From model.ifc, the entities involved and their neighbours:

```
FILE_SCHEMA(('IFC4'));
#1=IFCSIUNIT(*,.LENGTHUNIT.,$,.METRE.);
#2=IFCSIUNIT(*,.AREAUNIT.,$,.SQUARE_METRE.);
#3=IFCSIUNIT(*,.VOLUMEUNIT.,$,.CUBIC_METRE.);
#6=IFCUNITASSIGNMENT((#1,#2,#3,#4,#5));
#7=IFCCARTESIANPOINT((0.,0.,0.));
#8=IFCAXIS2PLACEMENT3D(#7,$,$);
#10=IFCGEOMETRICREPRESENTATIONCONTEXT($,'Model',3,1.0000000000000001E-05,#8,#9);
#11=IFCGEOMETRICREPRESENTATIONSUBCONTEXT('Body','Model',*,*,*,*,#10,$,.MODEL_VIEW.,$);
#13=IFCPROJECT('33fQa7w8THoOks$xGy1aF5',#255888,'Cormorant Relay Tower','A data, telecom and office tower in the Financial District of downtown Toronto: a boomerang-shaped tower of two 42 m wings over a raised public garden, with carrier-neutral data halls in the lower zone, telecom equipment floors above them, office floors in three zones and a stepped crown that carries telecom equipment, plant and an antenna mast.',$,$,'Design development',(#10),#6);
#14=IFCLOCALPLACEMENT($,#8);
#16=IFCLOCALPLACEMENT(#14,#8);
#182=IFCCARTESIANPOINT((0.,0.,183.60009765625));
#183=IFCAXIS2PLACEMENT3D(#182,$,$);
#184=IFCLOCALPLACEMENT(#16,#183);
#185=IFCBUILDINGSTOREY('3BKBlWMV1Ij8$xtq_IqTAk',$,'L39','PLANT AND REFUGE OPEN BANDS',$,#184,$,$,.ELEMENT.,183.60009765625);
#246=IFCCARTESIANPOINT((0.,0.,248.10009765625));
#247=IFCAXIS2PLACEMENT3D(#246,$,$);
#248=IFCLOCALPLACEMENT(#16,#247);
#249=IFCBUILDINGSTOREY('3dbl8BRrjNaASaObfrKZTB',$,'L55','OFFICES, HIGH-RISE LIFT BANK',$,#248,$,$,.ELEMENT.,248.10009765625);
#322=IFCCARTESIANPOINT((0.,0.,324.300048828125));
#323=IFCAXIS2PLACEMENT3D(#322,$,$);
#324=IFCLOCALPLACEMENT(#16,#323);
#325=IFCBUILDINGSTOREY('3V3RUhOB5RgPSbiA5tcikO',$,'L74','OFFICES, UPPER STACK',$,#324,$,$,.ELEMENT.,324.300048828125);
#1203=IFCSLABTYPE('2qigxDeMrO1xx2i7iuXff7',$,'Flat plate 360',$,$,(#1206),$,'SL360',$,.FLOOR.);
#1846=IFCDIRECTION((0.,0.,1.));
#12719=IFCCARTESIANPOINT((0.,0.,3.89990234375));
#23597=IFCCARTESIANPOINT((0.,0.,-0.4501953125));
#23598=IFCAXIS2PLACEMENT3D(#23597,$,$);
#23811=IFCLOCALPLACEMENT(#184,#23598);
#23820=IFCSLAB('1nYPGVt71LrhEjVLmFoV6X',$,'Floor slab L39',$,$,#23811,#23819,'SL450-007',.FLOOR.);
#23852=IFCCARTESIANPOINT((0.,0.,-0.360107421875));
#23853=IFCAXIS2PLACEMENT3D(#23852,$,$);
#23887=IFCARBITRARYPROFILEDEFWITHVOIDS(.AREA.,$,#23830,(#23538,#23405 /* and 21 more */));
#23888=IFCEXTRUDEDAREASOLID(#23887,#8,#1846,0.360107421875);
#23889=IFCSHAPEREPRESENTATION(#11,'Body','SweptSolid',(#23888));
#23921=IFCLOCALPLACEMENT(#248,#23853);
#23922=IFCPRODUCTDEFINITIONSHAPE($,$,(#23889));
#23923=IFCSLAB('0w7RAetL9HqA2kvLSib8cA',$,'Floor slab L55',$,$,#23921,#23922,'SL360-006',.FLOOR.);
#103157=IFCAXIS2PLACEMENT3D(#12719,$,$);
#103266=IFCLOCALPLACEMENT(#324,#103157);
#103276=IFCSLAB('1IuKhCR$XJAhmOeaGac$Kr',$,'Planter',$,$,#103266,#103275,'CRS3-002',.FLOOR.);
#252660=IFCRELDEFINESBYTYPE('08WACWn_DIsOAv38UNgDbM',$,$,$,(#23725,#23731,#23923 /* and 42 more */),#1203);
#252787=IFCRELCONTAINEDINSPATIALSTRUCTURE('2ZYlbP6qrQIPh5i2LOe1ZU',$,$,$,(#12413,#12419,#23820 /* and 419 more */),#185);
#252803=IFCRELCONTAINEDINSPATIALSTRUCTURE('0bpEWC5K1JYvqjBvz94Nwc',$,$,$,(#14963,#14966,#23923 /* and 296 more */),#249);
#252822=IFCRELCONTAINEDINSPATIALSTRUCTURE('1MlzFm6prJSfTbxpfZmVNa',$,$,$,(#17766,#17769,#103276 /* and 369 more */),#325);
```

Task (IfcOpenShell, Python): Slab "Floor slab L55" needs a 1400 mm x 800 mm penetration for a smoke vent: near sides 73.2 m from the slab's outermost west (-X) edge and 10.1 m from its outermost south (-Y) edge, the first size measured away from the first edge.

```python
import numpy as np
import ifcopenshell
import ifcopenshell.api.feature
import ifcopenshell.api.geometry
import ifcopenshell.api.root
import ifcopenshell.geom
import ifcopenshell.util.placement
import ifcopenshell.util.representation
import ifcopenshell.util.shape
import ifcopenshell.util.unit

model = ifcopenshell.open("model.ifc")
unit_scale = ifcopenshell.util.unit.calculate_unit_scale(model)
settings = ifcopenshell.geom.settings()


def volume(element):
    """Net volume in cubic metres, openings subtracted."""
    shape = ifcopenshell.geom.create_shape(settings, element)
    return ifcopenshell.util.shape.get_volume(shape.geometry)


slab = model.by_guid("0w7RAetL9HqA2kvLSib8cA")
before = volume(slab)

# Extent in the slab's own axes, in metres. The edges named are its -X and -Y sides.
slab_shape = ifcopenshell.geom.create_shape(settings, slab)
vertices = ifcopenshell.util.shape.get_vertices(slab_shape.geometry)
x_min, y_min, bottom = vertices.min(axis=0)
top = vertices[:, 2].max()

opening = ifcopenshell.api.root.create_entity(model, ifc_class="IfcOpeningElement", name="Smoke vent opening", predefined_type="OPENING")
context = ifcopenshell.util.representation.get_context(model, "Model", "Body", "MODEL_VIEW")
width, depth = 1.4, 0.8
outline = [(0.0, 0.0), (width, 0.0), (width, depth), (0.0, depth), (0.0, 0.0)]
# Overshoot both faces by 50 mm so the cut is clean.
shape = ifcopenshell.api.geometry.add_slab_representation(
    model, context=context, depth=top - bottom + 0.1, polyline=outline
)
ifcopenshell.api.geometry.assign_representation(model, product=opening, representation=shape)

matrix = ifcopenshell.util.placement.get_local_placement(slab.ObjectPlacement)
matrix[:, 3] = matrix @ np.append(np.array([x_min + 73.2, y_min + 10.1, bottom - 0.05]) / unit_scale, 1.0)
ifcopenshell.api.geometry.edit_object_placement(model, product=opening, matrix=matrix, is_si=False)
ifcopenshell.api.feature.add_feature(model, feature=opening, element=slab)

after = volume(slab)

print(f"slab volume {before:.3f} -> {after:.3f} m3")

model.write("model_edited.ifc")
```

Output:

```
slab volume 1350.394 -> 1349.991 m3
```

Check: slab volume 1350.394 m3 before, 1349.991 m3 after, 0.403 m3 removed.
